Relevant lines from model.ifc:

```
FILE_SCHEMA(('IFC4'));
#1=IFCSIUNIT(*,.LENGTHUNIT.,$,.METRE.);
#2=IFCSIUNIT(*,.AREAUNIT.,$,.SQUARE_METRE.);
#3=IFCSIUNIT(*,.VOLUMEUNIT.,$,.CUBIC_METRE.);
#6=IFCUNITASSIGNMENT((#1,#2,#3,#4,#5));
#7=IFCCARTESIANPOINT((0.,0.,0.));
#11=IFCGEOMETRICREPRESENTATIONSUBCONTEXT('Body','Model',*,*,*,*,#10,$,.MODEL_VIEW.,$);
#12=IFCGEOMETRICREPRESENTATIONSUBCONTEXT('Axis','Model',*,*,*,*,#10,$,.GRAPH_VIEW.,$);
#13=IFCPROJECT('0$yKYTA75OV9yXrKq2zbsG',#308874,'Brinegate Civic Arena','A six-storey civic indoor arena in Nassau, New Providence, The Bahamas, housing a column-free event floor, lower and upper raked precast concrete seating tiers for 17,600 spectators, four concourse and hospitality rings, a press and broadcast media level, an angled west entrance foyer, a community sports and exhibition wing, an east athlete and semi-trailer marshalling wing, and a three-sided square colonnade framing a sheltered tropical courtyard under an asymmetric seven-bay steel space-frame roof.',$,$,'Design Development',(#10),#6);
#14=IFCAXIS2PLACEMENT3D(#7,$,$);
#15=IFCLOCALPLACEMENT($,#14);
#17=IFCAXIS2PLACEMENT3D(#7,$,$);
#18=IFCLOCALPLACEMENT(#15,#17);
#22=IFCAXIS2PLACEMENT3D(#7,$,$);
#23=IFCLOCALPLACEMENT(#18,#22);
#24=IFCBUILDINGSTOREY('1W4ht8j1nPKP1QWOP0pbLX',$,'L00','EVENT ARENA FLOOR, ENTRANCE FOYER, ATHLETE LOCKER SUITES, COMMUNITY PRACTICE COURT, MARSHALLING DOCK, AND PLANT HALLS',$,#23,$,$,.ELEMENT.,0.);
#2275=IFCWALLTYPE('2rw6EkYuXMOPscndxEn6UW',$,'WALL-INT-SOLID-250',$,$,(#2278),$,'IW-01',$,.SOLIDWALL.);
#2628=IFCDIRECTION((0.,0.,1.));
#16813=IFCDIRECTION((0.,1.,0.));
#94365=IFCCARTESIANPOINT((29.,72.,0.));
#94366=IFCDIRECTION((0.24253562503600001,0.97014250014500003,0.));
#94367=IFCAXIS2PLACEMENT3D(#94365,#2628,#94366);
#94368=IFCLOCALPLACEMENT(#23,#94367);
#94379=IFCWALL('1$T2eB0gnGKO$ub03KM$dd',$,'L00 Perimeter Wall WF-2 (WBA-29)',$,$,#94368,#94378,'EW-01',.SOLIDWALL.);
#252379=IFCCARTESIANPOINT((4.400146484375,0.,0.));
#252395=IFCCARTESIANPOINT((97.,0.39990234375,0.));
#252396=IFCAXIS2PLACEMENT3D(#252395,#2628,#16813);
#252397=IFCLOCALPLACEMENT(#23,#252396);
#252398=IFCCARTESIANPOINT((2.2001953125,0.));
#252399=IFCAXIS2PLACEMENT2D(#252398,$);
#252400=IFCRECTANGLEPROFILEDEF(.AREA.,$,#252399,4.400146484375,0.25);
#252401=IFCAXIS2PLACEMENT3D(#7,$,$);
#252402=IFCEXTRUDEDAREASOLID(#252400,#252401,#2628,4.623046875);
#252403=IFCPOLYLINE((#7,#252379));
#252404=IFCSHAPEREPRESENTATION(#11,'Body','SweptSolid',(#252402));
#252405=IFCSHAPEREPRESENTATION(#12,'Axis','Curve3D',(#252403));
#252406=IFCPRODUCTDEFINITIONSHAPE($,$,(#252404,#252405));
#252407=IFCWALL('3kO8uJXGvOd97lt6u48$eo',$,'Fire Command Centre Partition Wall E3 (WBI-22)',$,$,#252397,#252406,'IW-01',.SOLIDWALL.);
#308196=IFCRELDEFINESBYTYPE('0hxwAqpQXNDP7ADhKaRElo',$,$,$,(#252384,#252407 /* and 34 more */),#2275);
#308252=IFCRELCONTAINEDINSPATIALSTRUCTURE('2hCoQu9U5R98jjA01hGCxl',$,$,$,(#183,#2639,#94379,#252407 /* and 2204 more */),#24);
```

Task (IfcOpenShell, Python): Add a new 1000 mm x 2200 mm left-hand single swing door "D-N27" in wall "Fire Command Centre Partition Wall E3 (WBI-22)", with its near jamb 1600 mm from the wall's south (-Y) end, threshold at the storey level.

```python
import numpy as np
import ifcopenshell
import ifcopenshell.api.feature
import ifcopenshell.api.geometry
import ifcopenshell.api.root
import ifcopenshell.api.spatial
import ifcopenshell.geom
import ifcopenshell.util.element
import ifcopenshell.util.placement
import ifcopenshell.util.representation
import ifcopenshell.util.shape
import ifcopenshell.util.unit

model = ifcopenshell.open("model.ifc")
unit_scale = ifcopenshell.util.unit.calculate_unit_scale(model)
settings = ifcopenshell.geom.settings()


def volume(element):
    """Net volume in cubic metres, openings subtracted."""
    shape = ifcopenshell.geom.create_shape(settings, element)
    return ifcopenshell.util.shape.get_volume(shape.geometry)


wall = model.by_id(252407)
storey = ifcopenshell.util.element.get_container(wall, ifc_class="IfcBuildingStorey")
context = ifcopenshell.util.representation.get_context(model, "Model", "Body", "MODEL_VIEW")
before = volume(wall)

width, height, from_end, sill = 1, 2.2, 1.6, 0.0  # metres

# The wall runs along its own X axis, and the end named is its -X end.
wall_shape = ifcopenshell.geom.create_shape(settings, wall)
x, y, z = ifcopenshell.util.shape.get_vertices(wall_shape.geometry).T
start = x.min() + from_end
face, thickness = float(y.min()), float(y.max() - y.min())
wall_matrix = ifcopenshell.util.placement.get_local_placement(wall.ObjectPlacement)
level = ifcopenshell.util.placement.get_local_placement(storey.ObjectPlacement)[2, 3]


def in_wall(x, y):
    """Placement at x, y metres in the wall's axes, at sill height."""
    matrix = wall_matrix.copy()
    matrix[:, 3] = wall_matrix @ np.array([x / unit_scale, y / unit_scale, 0.0, 1.0])
    matrix[2, 3] = level + sill / unit_scale
    return matrix


# Opening: a box that overshoots both wall faces by 50 mm.
opening = ifcopenshell.api.root.create_entity(model, ifc_class="IfcOpeningElement", predefined_type="OPENING")
box = ifcopenshell.api.geometry.add_wall_representation(
    model, context=context, length=width, height=height, thickness=thickness + 0.1
)
ifcopenshell.api.geometry.assign_representation(model, product=opening, representation=box)
ifcopenshell.api.geometry.edit_object_placement(model, product=opening, matrix=in_wall(start, face - 0.05), is_si=False)
ifcopenshell.api.feature.add_feature(model, feature=opening, element=wall)

door = ifcopenshell.api.root.create_entity(model, ifc_class="IfcDoor", name="D-N27", predefined_type="DOOR")
door.OverallWidth, door.OverallHeight = width / unit_scale, height / unit_scale
door.OperationType = "SINGLE_SWING_LEFT"
body = ifcopenshell.api.geometry.add_door_representation(
    model,
    context=context,
    overall_width=door.OverallWidth,
    overall_height=door.OverallHeight,
    operation_type="SINGLE_SWING_LEFT",
    lining_properties={"LiningDepth": thickness / unit_scale, "ThresholdDepth": thickness / unit_scale},
)
ifcopenshell.api.geometry.assign_representation(model, product=door, representation=body)
ifcopenshell.api.spatial.assign_container(model, products=[door], relating_structure=storey)
ifcopenshell.api.feature.add_filling(model, opening=opening, element=door)

# The lining spans the wall, so the door starts at the wall face.
ifcopenshell.api.geometry.edit_object_placement(model, product=door, matrix=in_wall(start, face), is_si=False)

after = volume(wall)

print(f"wall volume {before:.3f} -> {after:.3f} m3")

model.write("model_rev.ifc")
```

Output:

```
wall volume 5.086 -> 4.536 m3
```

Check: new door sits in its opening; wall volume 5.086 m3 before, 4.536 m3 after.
